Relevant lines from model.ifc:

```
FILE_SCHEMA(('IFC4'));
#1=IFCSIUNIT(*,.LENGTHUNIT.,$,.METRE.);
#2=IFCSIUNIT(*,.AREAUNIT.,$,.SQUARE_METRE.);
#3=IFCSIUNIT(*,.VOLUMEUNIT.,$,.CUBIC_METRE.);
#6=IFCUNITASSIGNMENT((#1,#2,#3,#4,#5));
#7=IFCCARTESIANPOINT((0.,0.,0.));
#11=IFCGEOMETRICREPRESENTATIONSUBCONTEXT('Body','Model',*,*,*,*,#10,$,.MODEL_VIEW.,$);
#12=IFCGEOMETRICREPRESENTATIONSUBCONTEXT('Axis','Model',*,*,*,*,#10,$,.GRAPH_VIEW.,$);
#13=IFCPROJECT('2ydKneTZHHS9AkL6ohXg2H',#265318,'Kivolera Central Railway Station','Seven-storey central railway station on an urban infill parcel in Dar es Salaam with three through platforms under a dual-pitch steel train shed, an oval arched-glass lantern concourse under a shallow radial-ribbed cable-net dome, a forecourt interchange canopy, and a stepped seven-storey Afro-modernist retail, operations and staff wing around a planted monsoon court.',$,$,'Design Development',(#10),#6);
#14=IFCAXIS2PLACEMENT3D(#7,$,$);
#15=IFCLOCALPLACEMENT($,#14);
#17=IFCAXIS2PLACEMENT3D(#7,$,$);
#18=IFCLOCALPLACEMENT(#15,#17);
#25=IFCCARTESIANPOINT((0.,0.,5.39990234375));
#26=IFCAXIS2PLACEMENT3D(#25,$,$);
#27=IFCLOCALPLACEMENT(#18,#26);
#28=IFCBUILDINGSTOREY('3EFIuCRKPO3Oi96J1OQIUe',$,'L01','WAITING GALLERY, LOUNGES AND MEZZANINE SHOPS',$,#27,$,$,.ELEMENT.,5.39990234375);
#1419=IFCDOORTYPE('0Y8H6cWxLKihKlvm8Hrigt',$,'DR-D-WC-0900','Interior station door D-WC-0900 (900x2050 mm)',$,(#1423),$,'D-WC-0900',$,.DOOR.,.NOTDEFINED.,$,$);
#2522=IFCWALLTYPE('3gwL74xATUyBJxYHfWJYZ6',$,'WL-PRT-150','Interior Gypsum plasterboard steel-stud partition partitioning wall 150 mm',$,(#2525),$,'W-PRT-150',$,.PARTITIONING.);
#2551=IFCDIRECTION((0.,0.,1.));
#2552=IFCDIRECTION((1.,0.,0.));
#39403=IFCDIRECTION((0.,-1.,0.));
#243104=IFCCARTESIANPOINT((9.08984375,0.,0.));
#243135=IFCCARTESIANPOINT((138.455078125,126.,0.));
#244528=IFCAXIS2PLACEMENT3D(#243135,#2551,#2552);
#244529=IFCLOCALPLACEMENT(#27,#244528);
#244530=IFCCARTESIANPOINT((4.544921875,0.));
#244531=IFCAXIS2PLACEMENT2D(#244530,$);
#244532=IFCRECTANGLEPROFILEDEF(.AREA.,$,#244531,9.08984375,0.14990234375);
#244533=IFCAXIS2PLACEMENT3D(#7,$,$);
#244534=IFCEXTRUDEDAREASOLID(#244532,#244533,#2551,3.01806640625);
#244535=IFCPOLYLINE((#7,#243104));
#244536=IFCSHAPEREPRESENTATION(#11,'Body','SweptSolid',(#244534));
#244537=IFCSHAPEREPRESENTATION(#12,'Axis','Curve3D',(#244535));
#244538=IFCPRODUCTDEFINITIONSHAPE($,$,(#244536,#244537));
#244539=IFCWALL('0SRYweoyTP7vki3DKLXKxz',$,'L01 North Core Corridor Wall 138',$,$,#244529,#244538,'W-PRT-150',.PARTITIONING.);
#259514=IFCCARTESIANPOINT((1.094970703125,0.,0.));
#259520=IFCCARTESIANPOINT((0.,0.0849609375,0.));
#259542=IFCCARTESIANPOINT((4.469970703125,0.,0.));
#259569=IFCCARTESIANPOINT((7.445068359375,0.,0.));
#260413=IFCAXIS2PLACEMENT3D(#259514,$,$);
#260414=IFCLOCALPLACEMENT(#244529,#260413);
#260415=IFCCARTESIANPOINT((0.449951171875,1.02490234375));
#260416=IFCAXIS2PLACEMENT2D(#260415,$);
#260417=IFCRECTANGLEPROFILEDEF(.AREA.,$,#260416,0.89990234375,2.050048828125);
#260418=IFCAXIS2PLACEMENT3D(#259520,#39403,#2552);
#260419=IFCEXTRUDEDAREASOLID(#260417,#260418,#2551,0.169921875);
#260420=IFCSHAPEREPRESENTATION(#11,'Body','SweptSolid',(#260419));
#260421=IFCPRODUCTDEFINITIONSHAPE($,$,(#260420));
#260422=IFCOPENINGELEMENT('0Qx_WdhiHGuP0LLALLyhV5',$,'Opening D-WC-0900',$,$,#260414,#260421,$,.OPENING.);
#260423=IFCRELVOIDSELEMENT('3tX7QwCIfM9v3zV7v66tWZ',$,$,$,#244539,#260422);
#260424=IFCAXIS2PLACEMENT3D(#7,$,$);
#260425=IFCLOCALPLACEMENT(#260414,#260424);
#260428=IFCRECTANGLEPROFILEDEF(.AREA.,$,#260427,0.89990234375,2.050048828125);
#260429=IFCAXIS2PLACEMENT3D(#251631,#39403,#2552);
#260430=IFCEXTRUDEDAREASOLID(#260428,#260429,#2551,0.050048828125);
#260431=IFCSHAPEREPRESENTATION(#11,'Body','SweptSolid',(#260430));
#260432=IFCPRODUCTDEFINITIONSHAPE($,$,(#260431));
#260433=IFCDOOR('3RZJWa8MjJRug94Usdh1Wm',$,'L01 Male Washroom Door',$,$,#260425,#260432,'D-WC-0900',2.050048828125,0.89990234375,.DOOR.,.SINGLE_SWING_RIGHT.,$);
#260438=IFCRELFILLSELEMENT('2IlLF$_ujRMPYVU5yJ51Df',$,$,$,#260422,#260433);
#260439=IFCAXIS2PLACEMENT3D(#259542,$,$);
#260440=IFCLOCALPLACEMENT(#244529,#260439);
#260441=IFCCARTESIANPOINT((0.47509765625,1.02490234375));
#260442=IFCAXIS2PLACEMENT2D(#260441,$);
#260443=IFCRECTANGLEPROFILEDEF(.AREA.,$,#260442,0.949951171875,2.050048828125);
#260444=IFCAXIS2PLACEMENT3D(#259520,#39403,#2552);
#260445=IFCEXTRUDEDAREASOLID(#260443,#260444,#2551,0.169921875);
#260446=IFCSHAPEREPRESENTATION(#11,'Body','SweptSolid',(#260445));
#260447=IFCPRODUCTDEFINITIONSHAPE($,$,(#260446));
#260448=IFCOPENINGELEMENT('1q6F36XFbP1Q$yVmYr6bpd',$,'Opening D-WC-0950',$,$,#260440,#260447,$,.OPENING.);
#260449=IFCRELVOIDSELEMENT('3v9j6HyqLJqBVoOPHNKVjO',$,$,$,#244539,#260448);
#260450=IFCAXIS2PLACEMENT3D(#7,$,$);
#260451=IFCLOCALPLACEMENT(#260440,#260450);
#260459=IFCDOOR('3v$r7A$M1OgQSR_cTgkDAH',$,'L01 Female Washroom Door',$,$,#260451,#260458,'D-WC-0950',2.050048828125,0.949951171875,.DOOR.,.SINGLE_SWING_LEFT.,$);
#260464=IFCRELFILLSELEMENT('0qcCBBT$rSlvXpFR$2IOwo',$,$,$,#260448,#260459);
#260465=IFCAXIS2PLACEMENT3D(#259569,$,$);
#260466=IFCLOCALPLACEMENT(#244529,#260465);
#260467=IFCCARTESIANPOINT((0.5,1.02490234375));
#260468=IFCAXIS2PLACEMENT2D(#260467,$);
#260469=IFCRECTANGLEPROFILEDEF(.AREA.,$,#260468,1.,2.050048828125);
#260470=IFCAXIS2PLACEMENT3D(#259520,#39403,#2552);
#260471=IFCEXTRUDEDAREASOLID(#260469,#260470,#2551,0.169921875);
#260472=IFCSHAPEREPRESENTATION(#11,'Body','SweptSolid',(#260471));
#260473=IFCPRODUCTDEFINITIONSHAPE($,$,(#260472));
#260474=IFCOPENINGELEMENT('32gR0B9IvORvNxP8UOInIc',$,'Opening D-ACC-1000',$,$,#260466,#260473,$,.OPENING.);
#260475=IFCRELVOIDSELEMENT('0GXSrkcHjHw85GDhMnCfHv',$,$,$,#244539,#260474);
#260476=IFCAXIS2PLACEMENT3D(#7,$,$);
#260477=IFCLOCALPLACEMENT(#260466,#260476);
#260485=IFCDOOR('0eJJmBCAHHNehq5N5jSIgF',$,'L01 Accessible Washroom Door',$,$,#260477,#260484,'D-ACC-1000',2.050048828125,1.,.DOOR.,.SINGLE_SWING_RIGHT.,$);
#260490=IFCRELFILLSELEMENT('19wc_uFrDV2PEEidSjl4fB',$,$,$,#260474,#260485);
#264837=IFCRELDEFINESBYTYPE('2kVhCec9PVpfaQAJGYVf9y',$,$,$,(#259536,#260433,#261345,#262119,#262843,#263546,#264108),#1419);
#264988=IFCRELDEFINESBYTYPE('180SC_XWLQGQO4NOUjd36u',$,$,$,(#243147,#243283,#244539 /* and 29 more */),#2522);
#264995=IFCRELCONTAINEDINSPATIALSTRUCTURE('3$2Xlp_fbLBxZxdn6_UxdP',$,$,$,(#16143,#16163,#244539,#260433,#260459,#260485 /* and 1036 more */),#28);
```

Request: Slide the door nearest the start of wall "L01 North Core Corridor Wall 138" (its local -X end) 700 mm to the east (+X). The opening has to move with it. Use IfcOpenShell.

```python
import ifcopenshell
import ifcopenshell.api.geometry
import ifcopenshell.util.placement

model = ifcopenshell.open("model.ifc")

door = model.by_id(260433)
opening = door.FillsVoids[0].RelatingOpeningElement
wall = opening.VoidsElements[0].RelatingBuildingElement

wall_matrix = ifcopenshell.util.placement.get_local_placement(wall.ObjectPlacement)
shift = wall_matrix[:3, 0] * 0.7
before = ifcopenshell.util.placement.get_local_placement(door.ObjectPlacement)[:3, 3].copy()

# The door is placed relative to its opening, so it follows when the opening moves.
matrix = ifcopenshell.util.placement.get_local_placement(opening.ObjectPlacement)
matrix[:3, 3] += shift
ifcopenshell.api.geometry.edit_object_placement(
    model, product=opening, matrix=matrix, is_si=False, should_transform_children=True
)

after = ifcopenshell.util.placement.get_local_placement(door.ObjectPlacement)[:3, 3]
print("door moved by", (after - before).round(3) + 0.0)

model.write("model_edited.ifc")
```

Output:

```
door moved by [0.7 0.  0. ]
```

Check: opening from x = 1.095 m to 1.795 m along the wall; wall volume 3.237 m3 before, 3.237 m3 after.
